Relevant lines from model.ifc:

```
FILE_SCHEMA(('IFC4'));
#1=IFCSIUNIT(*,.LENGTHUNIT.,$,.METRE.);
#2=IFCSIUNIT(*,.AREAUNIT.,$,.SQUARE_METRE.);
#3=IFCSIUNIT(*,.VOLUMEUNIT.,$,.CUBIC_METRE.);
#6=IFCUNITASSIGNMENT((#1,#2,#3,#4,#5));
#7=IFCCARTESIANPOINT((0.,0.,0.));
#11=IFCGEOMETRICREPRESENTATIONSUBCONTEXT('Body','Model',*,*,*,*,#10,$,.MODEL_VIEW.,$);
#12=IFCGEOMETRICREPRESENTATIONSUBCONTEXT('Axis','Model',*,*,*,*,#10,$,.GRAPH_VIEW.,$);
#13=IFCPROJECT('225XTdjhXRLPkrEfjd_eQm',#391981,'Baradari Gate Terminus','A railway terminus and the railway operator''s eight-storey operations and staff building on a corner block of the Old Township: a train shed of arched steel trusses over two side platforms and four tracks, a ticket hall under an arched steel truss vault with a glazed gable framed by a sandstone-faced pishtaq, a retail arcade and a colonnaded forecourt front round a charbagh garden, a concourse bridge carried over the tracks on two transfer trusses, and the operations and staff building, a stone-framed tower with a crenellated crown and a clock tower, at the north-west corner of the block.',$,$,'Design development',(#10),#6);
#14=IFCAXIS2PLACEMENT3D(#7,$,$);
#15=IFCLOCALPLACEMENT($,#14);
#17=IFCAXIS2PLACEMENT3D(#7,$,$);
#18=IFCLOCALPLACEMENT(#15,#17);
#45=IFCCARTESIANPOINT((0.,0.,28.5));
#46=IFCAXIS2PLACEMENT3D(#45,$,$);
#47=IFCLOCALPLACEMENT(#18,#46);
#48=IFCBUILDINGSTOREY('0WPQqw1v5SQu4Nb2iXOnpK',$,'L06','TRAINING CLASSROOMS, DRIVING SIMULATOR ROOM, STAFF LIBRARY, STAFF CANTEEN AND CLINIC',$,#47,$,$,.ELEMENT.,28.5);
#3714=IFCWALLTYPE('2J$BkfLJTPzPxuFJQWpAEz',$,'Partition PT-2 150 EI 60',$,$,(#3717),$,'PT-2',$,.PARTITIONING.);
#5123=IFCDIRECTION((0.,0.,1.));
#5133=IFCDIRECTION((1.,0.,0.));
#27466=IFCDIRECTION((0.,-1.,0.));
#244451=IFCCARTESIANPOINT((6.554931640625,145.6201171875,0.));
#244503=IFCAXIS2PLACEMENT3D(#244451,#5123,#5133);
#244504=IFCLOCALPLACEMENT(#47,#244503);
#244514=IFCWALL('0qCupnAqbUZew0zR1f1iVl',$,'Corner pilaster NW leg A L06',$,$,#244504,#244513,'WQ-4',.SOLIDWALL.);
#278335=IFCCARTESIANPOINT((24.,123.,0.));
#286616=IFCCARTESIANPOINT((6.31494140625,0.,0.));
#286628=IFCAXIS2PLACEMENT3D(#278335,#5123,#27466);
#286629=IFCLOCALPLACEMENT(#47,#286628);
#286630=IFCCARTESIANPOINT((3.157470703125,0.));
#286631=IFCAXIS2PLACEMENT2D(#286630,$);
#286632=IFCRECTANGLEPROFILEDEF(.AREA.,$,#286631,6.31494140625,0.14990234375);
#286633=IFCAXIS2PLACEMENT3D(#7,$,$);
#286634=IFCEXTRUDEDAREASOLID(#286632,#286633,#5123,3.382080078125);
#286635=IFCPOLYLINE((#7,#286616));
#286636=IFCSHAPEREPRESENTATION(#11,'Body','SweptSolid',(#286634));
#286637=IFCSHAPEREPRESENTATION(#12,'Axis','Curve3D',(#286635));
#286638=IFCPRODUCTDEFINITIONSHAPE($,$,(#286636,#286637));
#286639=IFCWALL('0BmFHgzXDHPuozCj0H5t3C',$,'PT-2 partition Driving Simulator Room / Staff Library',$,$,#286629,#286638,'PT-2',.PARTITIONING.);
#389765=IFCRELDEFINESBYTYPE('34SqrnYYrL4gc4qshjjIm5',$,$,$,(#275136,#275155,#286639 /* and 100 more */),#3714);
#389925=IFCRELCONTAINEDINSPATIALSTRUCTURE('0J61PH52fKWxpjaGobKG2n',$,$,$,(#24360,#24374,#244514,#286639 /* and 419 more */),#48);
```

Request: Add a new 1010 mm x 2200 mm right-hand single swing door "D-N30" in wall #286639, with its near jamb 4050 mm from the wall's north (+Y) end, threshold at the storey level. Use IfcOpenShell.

```python
import numpy as np
import ifcopenshell
import ifcopenshell.api.feature
import ifcopenshell.api.geometry
import ifcopenshell.api.root
import ifcopenshell.api.spatial
import ifcopenshell.geom
import ifcopenshell.util.element
import ifcopenshell.util.placement
import ifcopenshell.util.representation
import ifcopenshell.util.shape
import ifcopenshell.util.unit

model = ifcopenshell.open("model.ifc")
unit_scale = ifcopenshell.util.unit.calculate_unit_scale(model)
settings = ifcopenshell.geom.settings()


def volume(element):
    """Net volume in cubic metres, openings subtracted."""
    shape = ifcopenshell.geom.create_shape(settings, element)
    return ifcopenshell.util.shape.get_volume(shape.geometry)


wall = model.by_guid("0BmFHgzXDHPuozCj0H5t3C")
storey = ifcopenshell.util.element.get_container(wall, ifc_class="IfcBuildingStorey")
context = ifcopenshell.util.representation.get_context(model, "Model", "Body", "MODEL_VIEW")
before = volume(wall)

width, height, from_end, sill = 1.01, 2.2, 4.05, 0.0  # metres

# The wall runs along its own X axis, and the end named is its -X end.
wall_shape = ifcopenshell.geom.create_shape(settings, wall)
x, y, z = ifcopenshell.util.shape.get_vertices(wall_shape.geometry).T
start = x.min() + from_end
face, thickness = float(y.min()), float(y.max() - y.min())
wall_matrix = ifcopenshell.util.placement.get_local_placement(wall.ObjectPlacement)
level = ifcopenshell.util.placement.get_local_placement(storey.ObjectPlacement)[2, 3]


def in_wall(x, y):
    """Placement at x, y metres in the wall's axes, at sill height."""
    matrix = wall_matrix.copy()
    matrix[:, 3] = wall_matrix @ np.array([x / unit_scale, y / unit_scale, 0.0, 1.0])
    matrix[2, 3] = level + sill / unit_scale
    return matrix


# Opening: a box that overshoots both wall faces by 50 mm.
opening = ifcopenshell.api.root.create_entity(model, ifc_class="IfcOpeningElement", predefined_type="OPENING")
box = ifcopenshell.api.geometry.add_wall_representation(
    model, context=context, length=width, height=height, thickness=thickness + 0.1
)
ifcopenshell.api.geometry.assign_representation(model, product=opening, representation=box)
ifcopenshell.api.geometry.edit_object_placement(model, product=opening, matrix=in_wall(start, face - 0.05), is_si=False)
ifcopenshell.api.feature.add_feature(model, feature=opening, element=wall)

door = ifcopenshell.api.root.create_entity(model, ifc_class="IfcDoor", name="D-N30", predefined_type="DOOR")
door.OverallWidth, door.OverallHeight = width / unit_scale, height / unit_scale
door.OperationType = "SINGLE_SWING_RIGHT"
body = ifcopenshell.api.geometry.add_door_representation(
    model,
    context=context,
    overall_width=door.OverallWidth,
    overall_height=door.OverallHeight,
    operation_type="SINGLE_SWING_RIGHT",
    lining_properties={"LiningDepth": thickness / unit_scale, "ThresholdDepth": thickness / unit_scale},
)
ifcopenshell.api.geometry.assign_representation(model, product=door, representation=body)
ifcopenshell.api.spatial.assign_container(model, products=[door], relating_structure=storey)
ifcopenshell.api.feature.add_filling(model, opening=opening, element=door)

# The lining spans the wall, so the door starts at the wall face.
ifcopenshell.api.geometry.edit_object_placement(model, product=door, matrix=in_wall(start, face), is_si=False)

after = volume(wall)

print(f"wall volume {before:.3f} -> {after:.3f} m3")

model.write("model_edited.ifc")
```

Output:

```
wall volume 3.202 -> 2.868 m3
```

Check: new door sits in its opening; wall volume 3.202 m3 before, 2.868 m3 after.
